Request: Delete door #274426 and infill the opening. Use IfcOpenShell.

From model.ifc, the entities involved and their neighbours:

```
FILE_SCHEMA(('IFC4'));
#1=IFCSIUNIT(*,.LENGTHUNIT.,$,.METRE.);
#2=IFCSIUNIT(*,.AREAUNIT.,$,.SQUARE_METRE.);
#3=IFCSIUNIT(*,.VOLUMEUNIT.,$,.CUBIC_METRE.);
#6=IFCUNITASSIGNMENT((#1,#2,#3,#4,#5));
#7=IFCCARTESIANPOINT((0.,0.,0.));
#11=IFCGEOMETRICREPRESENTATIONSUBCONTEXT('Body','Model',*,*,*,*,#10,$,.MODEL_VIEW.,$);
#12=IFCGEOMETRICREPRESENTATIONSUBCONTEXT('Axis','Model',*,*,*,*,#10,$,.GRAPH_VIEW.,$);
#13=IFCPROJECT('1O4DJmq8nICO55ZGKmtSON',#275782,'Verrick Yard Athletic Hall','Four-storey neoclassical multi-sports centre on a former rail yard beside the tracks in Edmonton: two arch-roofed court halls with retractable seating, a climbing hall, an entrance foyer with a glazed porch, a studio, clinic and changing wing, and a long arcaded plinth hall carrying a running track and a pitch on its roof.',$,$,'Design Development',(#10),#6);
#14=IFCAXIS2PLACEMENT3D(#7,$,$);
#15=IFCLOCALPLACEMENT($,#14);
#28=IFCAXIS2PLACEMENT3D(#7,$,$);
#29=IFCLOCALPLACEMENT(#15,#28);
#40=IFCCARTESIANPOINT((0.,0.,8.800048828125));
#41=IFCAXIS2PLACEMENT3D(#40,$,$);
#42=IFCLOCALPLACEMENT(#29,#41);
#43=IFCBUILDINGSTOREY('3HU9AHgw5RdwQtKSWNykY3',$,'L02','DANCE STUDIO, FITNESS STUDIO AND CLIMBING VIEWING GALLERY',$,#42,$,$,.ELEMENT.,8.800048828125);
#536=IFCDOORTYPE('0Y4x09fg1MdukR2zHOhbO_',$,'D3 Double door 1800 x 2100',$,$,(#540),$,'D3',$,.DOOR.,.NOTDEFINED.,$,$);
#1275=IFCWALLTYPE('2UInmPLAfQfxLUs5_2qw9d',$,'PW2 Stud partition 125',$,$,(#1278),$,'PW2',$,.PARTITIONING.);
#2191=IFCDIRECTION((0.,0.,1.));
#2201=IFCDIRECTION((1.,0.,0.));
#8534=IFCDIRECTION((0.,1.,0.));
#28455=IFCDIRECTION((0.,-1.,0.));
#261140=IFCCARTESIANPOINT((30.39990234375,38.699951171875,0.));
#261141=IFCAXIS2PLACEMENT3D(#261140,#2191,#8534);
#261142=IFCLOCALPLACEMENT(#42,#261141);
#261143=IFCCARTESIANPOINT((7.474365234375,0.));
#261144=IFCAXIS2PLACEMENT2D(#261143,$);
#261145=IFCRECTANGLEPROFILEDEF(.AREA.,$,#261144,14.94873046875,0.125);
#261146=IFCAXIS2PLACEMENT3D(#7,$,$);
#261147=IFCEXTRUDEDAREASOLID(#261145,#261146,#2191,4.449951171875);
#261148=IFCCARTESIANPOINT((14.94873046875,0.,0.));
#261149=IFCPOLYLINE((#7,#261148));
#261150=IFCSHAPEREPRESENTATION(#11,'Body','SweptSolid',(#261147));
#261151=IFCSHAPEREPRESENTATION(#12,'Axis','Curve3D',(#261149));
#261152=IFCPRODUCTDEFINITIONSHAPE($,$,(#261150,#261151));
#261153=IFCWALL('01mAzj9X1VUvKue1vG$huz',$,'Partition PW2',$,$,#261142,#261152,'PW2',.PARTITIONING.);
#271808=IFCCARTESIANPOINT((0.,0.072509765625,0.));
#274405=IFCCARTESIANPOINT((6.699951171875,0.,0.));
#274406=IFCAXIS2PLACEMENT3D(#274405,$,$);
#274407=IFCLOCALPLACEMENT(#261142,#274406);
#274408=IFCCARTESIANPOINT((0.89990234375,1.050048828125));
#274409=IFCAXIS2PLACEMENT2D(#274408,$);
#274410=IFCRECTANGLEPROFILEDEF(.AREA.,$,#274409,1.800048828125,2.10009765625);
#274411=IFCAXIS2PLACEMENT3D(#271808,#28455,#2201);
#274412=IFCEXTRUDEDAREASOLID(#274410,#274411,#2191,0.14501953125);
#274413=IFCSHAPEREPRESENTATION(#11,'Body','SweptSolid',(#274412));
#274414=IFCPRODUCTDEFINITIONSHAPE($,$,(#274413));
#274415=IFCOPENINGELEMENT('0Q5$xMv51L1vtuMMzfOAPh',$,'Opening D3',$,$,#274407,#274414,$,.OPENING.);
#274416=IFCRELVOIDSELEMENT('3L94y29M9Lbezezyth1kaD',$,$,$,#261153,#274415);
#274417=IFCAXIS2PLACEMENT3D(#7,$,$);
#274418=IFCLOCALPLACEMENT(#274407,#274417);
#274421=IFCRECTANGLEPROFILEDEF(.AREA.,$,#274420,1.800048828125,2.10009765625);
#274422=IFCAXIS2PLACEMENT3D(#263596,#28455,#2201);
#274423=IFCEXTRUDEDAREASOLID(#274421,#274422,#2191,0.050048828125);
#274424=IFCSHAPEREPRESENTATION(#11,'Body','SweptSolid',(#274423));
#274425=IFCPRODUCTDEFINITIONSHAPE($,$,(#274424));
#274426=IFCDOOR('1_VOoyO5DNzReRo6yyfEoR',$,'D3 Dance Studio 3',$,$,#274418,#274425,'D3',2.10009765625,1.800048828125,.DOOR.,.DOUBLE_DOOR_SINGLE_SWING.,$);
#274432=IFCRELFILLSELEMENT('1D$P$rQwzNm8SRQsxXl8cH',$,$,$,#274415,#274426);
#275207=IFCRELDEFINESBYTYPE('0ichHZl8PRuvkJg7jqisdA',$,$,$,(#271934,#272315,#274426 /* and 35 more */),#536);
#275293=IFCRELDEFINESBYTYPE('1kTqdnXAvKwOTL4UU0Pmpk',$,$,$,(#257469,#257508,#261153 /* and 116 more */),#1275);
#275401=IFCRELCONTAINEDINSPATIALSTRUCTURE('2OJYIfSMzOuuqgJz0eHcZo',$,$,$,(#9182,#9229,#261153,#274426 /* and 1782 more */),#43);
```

```python
import ifcopenshell
import ifcopenshell.api.feature
import ifcopenshell.api.root
import ifcopenshell.geom
import ifcopenshell.util.shape

model = ifcopenshell.open("model.ifc")
settings = ifcopenshell.geom.settings()


def volume(element):
    """Net volume in cubic metres, openings subtracted."""
    shape = ifcopenshell.geom.create_shape(settings, element)
    return ifcopenshell.util.shape.get_volume(shape.geometry)


door = model.by_guid("1_VOoyO5DNzReRo6yyfEoR")
opening = door.FillsVoids[0].RelatingOpeningElement
wall = opening.VoidsElements[0].RelatingBuildingElement
before = volume(wall)

ifcopenshell.api.root.remove_product(model, product=door)
ifcopenshell.api.feature.remove_feature(model, feature=opening)

after = volume(wall)

print(f"wall volume {before:.3f} -> {after:.3f} m3")

model.write("model-out.ifc")
```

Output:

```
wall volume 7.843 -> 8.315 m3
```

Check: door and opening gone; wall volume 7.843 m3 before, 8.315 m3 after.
